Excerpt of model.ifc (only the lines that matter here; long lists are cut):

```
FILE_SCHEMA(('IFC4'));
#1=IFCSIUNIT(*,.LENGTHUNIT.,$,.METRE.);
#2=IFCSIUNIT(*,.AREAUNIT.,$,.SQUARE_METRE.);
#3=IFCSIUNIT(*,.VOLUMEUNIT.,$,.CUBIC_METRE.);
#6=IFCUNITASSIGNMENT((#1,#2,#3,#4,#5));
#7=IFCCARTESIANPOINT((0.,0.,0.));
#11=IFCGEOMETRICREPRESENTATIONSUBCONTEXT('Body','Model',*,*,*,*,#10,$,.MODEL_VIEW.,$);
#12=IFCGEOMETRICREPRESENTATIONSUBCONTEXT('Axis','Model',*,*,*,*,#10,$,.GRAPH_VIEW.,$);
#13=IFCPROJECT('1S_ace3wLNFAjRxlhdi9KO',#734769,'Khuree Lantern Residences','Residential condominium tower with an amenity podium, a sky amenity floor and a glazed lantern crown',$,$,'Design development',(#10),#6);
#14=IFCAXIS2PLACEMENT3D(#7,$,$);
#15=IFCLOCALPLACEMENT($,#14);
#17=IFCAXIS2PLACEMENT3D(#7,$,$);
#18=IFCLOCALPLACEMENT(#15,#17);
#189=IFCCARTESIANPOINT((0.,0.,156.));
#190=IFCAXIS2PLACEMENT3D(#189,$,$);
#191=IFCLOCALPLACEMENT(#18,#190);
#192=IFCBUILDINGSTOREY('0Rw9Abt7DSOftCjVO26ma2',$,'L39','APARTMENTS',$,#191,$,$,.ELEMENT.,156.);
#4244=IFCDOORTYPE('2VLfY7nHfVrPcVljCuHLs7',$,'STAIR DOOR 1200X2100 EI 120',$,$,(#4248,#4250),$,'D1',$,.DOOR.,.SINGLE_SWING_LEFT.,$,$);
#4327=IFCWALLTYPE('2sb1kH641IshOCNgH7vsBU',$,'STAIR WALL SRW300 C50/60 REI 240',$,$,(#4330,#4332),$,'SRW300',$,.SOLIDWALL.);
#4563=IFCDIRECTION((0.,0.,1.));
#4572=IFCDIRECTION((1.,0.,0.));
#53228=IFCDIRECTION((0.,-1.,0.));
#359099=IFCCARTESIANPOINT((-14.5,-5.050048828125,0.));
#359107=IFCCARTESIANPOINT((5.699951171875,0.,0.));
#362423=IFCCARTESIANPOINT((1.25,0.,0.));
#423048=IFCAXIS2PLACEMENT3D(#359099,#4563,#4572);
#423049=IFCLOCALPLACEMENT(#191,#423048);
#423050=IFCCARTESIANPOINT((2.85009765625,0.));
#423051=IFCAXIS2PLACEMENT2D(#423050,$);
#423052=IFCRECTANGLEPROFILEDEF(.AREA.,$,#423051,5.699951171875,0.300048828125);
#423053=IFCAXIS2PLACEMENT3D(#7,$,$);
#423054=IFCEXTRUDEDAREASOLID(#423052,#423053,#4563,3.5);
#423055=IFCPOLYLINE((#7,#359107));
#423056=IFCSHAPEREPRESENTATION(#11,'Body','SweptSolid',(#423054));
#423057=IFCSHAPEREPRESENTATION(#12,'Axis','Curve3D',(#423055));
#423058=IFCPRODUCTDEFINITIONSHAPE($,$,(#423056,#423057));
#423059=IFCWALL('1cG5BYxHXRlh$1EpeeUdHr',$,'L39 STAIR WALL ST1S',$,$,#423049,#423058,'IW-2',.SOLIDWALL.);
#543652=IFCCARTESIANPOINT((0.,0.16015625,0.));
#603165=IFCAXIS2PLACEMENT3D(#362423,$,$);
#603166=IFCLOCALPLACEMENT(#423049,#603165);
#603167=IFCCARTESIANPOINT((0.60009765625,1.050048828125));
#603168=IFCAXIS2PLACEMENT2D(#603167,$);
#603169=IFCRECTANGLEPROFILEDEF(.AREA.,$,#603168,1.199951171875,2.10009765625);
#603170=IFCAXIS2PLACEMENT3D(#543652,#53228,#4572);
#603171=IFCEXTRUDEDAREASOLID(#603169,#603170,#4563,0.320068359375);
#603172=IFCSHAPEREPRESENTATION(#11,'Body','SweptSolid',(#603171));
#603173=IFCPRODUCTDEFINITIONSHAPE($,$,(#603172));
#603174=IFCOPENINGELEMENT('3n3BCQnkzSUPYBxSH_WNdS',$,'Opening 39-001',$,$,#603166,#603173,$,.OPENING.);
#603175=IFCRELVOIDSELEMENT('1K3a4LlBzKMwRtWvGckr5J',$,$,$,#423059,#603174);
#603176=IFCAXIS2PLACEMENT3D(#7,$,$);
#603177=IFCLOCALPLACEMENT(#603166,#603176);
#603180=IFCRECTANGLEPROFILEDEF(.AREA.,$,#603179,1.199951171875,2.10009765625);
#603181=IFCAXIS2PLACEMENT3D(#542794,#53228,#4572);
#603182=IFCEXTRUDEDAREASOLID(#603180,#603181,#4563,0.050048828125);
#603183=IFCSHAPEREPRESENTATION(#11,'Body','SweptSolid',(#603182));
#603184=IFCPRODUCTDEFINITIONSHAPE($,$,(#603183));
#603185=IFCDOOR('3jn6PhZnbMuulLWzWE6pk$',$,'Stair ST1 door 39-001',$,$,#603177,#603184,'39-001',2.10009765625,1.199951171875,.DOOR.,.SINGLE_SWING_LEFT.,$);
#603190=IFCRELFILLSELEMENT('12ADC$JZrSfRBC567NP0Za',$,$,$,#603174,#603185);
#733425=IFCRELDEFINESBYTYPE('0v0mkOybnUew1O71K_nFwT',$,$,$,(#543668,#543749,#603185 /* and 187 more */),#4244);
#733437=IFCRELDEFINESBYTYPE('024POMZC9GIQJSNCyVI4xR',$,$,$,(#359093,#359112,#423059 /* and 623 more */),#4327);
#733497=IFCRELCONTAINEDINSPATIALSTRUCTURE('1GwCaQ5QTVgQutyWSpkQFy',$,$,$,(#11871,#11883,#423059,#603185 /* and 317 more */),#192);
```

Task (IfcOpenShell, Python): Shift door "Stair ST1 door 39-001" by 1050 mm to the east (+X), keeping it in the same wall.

```python
import ifcopenshell
import ifcopenshell.api.geometry
import ifcopenshell.util.placement
import ifcopenshell.util.unit

model = ifcopenshell.open("model.ifc")
unit_scale = ifcopenshell.util.unit.calculate_unit_scale(model)

door = model.by_id(603185)
opening = door.FillsVoids[0].RelatingOpeningElement
wall = opening.VoidsElements[0].RelatingBuildingElement

wall_matrix = ifcopenshell.util.placement.get_local_placement(wall.ObjectPlacement)
shift = wall_matrix[:3, 0] * 1.05 / unit_scale
before = ifcopenshell.util.placement.get_local_placement(door.ObjectPlacement)[:3, 3].copy()

# The door is placed relative to its opening, so it follows when the opening moves.
matrix = ifcopenshell.util.placement.get_local_placement(opening.ObjectPlacement)
matrix[:3, 3] += shift
ifcopenshell.api.geometry.edit_object_placement(
    model, product=opening, matrix=matrix, is_si=False, should_transform_children=True
)

after = ifcopenshell.util.placement.get_local_placement(door.ObjectPlacement)[:3, 3]
print("door moved by", (after - before).round(3) + 0.0)

model.write("model_v2.ifc")
```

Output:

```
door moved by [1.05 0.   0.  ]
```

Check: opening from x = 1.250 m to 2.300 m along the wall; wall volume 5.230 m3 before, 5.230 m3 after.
